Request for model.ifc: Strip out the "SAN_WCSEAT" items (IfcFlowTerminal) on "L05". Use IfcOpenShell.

First a look at what the model holds.

```python
import ifcopenshell
import ifcopenshell.util.element

model = ifcopenshell.open("model.ifc")
print(model.schema)
storey = next(s for s in model.by_type("IfcBuildingStorey") if s.Name == "L05")
terminals = [e for e in ifcopenshell.util.element.get_decomposition(storey) if e.is_a("IfcFlowTerminal")]
seen = {}
for e in terminals:
    element_type = ifcopenshell.util.element.get_type(e)
    name = element_type.Name if element_type not in (None, e) else None
    seen[name] = seen.get(name, 0) + 1
for name, count in sorted(seen.items(), key=str):
    print(count, "x", name)
```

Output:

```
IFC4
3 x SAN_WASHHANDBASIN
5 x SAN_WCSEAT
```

```python
import ifcopenshell
import ifcopenshell.api.root
import ifcopenshell.util.element

model = ifcopenshell.open("model.ifc")

storey = next(s for s in model.by_type("IfcBuildingStorey") if s.Name == "L05")
terminals = [e for e in ifcopenshell.util.element.get_decomposition(storey) if e.is_a("IfcFlowTerminal")]
targets = [e for e in terminals if (t := ifcopenshell.util.element.get_type(e)) not in (None, e) and t.Name == "SAN_WCSEAT"]

for e in targets:
    ifcopenshell.api.root.remove_product(model, product=e)
print(len(targets), "removed")

model.write("model_rev.ifc")
```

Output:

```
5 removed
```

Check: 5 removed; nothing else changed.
